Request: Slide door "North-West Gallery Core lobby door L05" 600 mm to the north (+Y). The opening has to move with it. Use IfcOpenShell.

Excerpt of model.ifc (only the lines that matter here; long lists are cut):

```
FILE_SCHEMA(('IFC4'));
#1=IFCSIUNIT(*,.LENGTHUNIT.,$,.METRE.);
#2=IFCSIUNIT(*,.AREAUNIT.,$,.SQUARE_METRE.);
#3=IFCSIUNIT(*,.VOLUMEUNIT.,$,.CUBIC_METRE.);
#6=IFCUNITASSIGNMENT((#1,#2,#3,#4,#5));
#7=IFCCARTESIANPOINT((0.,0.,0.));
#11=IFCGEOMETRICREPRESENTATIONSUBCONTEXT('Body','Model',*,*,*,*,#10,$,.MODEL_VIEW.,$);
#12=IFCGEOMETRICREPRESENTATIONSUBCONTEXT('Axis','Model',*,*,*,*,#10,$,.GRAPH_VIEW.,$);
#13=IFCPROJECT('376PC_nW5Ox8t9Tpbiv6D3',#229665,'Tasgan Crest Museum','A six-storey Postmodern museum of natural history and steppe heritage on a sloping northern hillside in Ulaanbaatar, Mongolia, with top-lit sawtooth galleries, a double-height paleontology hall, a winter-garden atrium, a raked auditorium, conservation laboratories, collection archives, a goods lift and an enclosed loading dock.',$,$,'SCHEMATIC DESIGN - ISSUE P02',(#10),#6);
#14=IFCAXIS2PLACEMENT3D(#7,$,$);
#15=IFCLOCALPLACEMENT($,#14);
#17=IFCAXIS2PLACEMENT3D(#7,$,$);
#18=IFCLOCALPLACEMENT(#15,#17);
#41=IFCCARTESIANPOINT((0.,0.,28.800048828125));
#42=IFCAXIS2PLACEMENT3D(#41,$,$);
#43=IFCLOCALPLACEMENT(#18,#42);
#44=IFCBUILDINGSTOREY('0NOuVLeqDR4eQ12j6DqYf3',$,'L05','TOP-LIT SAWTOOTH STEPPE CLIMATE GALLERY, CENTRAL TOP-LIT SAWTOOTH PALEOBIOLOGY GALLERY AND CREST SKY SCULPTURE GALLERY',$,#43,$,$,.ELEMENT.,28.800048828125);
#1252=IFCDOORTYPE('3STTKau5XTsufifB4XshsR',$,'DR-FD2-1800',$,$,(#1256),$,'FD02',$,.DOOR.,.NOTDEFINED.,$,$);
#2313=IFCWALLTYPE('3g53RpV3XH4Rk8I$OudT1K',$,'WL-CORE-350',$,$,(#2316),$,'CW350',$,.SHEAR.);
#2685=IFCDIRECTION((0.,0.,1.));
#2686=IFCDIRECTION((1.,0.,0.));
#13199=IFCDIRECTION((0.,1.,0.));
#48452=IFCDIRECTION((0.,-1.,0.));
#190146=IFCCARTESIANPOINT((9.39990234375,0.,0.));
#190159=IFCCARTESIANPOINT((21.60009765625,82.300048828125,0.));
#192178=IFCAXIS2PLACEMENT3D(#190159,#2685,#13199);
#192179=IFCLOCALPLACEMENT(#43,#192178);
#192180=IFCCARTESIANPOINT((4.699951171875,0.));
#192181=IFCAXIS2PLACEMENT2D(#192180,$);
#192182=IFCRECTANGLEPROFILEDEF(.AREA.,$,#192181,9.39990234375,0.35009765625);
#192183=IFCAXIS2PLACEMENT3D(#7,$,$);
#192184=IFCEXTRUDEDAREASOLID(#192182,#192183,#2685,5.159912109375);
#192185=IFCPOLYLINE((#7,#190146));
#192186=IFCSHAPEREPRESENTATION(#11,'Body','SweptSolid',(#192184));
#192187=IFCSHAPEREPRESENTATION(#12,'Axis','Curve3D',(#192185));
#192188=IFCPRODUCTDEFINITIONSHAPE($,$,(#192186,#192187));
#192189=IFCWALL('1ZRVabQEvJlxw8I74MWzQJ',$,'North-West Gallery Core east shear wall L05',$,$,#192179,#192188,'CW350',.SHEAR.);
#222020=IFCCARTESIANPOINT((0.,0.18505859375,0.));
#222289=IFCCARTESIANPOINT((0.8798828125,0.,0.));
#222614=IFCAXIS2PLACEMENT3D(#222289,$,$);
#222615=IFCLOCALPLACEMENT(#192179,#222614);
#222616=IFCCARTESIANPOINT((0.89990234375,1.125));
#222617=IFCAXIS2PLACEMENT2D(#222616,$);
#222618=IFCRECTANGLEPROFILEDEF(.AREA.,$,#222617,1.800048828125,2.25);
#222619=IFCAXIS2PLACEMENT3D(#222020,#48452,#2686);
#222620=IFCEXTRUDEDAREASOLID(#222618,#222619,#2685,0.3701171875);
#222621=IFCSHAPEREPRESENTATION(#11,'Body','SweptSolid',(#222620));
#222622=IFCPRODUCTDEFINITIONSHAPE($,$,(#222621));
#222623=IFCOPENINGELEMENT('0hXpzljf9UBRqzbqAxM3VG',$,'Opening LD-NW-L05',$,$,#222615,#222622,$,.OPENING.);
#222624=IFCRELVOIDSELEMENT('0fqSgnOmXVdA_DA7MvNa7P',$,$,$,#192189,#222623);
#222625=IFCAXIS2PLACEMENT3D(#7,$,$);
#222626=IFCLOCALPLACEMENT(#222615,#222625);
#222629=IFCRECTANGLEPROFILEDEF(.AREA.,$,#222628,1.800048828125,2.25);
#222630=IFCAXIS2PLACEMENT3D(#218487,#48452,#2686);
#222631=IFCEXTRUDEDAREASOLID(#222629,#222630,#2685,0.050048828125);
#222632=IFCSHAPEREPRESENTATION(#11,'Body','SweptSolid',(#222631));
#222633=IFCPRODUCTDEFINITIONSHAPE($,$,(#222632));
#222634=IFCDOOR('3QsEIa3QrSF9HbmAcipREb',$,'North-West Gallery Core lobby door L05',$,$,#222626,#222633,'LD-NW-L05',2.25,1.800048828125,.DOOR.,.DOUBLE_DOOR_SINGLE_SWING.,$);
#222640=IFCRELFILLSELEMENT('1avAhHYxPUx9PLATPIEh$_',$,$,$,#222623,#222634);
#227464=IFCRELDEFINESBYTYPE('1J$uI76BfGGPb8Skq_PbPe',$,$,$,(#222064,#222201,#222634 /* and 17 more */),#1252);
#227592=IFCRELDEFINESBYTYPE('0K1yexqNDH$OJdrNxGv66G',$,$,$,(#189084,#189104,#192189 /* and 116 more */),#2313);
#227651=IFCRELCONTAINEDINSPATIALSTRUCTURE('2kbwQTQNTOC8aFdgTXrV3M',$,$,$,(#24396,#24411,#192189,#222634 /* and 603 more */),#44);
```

```python
import ifcopenshell
import ifcopenshell.api.geometry
import ifcopenshell.util.placement
import ifcopenshell.util.unit

model = ifcopenshell.open("model.ifc")
unit_scale = ifcopenshell.util.unit.calculate_unit_scale(model)

door = model.by_guid("3QsEIa3QrSF9HbmAcipREb")
opening = door.FillsVoids[0].RelatingOpeningElement
wall = opening.VoidsElements[0].RelatingBuildingElement

wall_matrix = ifcopenshell.util.placement.get_local_placement(wall.ObjectPlacement)
shift = wall_matrix[:3, 0] * 0.6 / unit_scale
before = ifcopenshell.util.placement.get_local_placement(door.ObjectPlacement)[:3, 3].copy()

# The door is placed relative to its opening, so it follows when the opening moves.
matrix = ifcopenshell.util.placement.get_local_placement(opening.ObjectPlacement)
matrix[:3, 3] += shift
ifcopenshell.api.geometry.edit_object_placement(
    model, product=opening, matrix=matrix, is_si=False, should_transform_children=True
)

after = ifcopenshell.util.placement.get_local_placement(door.ObjectPlacement)[:3, 3]
print("door moved by", (after - before).round(3) + 0.0)

model.write("model_updated.ifc")
```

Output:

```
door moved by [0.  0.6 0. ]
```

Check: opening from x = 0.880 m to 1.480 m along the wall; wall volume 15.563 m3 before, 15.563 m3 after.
